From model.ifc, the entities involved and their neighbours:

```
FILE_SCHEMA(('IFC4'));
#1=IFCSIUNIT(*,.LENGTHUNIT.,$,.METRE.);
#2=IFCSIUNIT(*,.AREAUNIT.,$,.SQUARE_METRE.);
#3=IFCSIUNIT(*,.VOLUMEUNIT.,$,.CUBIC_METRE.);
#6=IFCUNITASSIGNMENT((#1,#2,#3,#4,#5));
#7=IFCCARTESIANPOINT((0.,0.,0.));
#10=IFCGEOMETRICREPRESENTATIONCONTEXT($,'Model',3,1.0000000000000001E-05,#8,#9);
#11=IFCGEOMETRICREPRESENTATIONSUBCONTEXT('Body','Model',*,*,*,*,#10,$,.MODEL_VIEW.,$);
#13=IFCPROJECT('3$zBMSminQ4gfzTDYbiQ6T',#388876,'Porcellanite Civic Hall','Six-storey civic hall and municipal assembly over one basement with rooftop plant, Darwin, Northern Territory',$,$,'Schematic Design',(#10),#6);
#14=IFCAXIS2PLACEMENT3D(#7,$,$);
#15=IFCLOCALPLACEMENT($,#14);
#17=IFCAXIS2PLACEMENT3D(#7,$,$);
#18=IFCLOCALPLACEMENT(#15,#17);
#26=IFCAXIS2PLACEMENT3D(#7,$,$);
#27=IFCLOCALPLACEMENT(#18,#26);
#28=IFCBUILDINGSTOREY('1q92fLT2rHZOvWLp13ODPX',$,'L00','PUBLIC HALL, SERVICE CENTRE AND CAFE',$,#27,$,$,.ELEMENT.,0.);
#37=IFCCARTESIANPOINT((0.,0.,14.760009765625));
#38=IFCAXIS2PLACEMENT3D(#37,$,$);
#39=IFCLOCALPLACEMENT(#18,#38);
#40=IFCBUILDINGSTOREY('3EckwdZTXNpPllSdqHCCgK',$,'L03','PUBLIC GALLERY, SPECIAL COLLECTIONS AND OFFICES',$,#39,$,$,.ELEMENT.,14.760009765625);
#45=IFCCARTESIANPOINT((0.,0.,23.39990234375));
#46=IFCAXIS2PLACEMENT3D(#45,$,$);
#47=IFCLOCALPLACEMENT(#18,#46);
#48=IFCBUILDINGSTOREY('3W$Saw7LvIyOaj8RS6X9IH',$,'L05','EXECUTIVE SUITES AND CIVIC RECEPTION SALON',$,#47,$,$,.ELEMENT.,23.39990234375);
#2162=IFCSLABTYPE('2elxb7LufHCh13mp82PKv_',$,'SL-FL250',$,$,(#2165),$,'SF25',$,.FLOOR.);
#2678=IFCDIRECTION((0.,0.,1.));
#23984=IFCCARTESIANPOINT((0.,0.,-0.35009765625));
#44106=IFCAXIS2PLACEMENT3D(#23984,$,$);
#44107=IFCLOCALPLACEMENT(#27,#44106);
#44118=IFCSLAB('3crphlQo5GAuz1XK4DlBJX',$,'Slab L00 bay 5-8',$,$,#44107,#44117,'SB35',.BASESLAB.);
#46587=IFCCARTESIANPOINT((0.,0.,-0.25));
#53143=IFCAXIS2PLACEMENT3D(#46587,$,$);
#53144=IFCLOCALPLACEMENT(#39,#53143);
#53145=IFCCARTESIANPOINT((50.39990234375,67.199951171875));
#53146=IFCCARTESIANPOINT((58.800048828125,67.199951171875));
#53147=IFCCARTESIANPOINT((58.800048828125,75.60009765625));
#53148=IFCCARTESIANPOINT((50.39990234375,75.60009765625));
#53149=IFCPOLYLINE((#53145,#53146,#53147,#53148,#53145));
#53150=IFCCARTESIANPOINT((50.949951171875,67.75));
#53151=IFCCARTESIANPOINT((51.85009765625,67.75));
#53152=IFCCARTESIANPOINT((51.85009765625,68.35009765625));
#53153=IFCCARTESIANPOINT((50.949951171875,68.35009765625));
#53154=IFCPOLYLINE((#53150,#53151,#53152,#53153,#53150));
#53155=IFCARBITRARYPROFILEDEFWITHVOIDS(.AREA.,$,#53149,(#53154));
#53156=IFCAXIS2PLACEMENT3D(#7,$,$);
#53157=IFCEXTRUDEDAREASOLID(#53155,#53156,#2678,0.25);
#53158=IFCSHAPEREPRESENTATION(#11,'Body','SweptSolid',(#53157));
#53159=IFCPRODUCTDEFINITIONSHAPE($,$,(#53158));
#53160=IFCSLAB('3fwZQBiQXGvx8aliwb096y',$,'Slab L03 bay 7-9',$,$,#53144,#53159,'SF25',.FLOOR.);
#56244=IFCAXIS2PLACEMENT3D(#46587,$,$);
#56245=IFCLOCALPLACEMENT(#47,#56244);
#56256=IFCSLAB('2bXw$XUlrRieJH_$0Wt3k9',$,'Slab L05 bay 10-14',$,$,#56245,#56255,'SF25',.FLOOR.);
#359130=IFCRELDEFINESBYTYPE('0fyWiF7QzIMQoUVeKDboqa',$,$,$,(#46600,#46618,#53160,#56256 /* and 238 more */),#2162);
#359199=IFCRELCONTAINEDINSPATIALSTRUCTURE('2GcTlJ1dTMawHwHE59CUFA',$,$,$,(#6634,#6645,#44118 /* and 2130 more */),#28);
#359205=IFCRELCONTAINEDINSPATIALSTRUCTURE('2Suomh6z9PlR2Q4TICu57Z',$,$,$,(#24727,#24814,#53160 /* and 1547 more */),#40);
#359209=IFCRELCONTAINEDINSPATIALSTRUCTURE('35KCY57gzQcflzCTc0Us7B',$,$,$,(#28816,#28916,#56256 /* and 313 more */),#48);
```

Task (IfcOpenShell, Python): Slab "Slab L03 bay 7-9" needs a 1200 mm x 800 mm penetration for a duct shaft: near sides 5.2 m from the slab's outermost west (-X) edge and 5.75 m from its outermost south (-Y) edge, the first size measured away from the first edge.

```python
import numpy as np
import ifcopenshell
import ifcopenshell.api.feature
import ifcopenshell.api.geometry
import ifcopenshell.api.root
import ifcopenshell.geom
import ifcopenshell.util.placement
import ifcopenshell.util.representation
import ifcopenshell.util.shape
import ifcopenshell.util.unit

model = ifcopenshell.open("model.ifc")
unit_scale = ifcopenshell.util.unit.calculate_unit_scale(model)
settings = ifcopenshell.geom.settings()


def volume(element):
    """Net volume in cubic metres, openings subtracted."""
    shape = ifcopenshell.geom.create_shape(settings, element)
    return ifcopenshell.util.shape.get_volume(shape.geometry)


slab = model.by_guid("3fwZQBiQXGvx8aliwb096y")
before = volume(slab)

# Extent in the slab's own axes, in metres. The edges named are its -X and -Y sides.
slab_shape = ifcopenshell.geom.create_shape(settings, slab)
vertices = ifcopenshell.util.shape.get_vertices(slab_shape.geometry)
x_min, y_min, bottom = vertices.min(axis=0)
top = vertices[:, 2].max()

opening = ifcopenshell.api.root.create_entity(model, ifc_class="IfcOpeningElement", name="Duct shaft opening", predefined_type="OPENING")
context = ifcopenshell.util.representation.get_context(model, "Model", "Body", "MODEL_VIEW")
width, depth = 1.2, 0.8
outline = [(0.0, 0.0), (width, 0.0), (width, depth), (0.0, depth), (0.0, 0.0)]
# Overshoot both faces by 50 mm so the cut is clean.
shape = ifcopenshell.api.geometry.add_slab_representation(
    model, context=context, depth=top - bottom + 0.1, polyline=outline
)
ifcopenshell.api.geometry.assign_representation(model, product=opening, representation=shape)

matrix = ifcopenshell.util.placement.get_local_placement(slab.ObjectPlacement)
matrix[:, 3] = matrix @ np.append(np.array([x_min + 5.2, y_min + 5.75, bottom - 0.05]) / unit_scale, 1.0)
ifcopenshell.api.geometry.edit_object_placement(model, product=opening, matrix=matrix, is_si=False)
ifcopenshell.api.feature.add_feature(model, feature=opening, element=slab)

after = volume(slab)

print(f"slab volume {before:.3f} -> {after:.3f} m3")

model.write("model_edited.ifc")
```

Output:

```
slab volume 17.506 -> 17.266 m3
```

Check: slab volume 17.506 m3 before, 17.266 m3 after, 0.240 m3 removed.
